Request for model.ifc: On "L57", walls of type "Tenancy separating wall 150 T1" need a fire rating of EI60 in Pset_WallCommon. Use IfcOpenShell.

First a look at what the model holds.

```python
import ifcopenshell
import ifcopenshell.util.element

model = ifcopenshell.open("model.ifc")
print(model.schema)
storey = next(s for s in model.by_type("IfcBuildingStorey") if s.Name == "L57")
walls = [e for e in ifcopenshell.util.element.get_decomposition(storey) if e.is_a("IfcWall")]
seen = {}
for e in walls:
    element_type = ifcopenshell.util.element.get_type(e)
    key = (element_type.Name if element_type != e and element_type else None, ifcopenshell.util.element.get_pset(e, "Pset_WallCommon", "FireRating"))
    seen[key] = seen.get(key, 0) + 1
for (name, value), count in sorted(seen.items(), key=str):
    print(count, "x", name, "|", value)
```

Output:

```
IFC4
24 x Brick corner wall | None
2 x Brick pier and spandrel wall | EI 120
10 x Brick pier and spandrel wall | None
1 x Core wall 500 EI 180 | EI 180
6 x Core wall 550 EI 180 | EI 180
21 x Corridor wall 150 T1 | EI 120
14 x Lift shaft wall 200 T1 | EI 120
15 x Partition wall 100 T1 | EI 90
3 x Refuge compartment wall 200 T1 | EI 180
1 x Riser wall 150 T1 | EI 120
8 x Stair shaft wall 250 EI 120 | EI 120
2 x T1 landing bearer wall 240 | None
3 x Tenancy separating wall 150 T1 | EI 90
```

```python
import ifcopenshell
import ifcopenshell.api.pset
import ifcopenshell.util.element

model = ifcopenshell.open("model.ifc")

storey = next(s for s in model.by_type("IfcBuildingStorey") if s.Name == "L57")
walls = [e for e in ifcopenshell.util.element.get_decomposition(storey) if e.is_a("IfcWall")]

count = 0
for e in walls:
    element_type = ifcopenshell.util.element.get_type(e)
    if element_type in (None, e) or element_type.Name != "Tenancy separating wall 150 T1":
        continue
    found = ifcopenshell.util.element.get_pset(e, "Pset_WallCommon", should_inherit=False)
    if found:
        pset = model.by_id(found["id"])
        if len(ifcopenshell.util.element.get_elements_by_pset(pset)) > 1:
            pset = ifcopenshell.api.pset.unshare_pset(model, products=[e], pset=pset)[0]
    else:
        pset = ifcopenshell.api.pset.add_pset(model, product=e, name="Pset_WallCommon")
    ifcopenshell.api.pset.edit_pset(model, pset=pset, properties={"FireRating": "EI60"})
    count += 1

print(count, "walls updated")

model.write("model_rev.ifc")
```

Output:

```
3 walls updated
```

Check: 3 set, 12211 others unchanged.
